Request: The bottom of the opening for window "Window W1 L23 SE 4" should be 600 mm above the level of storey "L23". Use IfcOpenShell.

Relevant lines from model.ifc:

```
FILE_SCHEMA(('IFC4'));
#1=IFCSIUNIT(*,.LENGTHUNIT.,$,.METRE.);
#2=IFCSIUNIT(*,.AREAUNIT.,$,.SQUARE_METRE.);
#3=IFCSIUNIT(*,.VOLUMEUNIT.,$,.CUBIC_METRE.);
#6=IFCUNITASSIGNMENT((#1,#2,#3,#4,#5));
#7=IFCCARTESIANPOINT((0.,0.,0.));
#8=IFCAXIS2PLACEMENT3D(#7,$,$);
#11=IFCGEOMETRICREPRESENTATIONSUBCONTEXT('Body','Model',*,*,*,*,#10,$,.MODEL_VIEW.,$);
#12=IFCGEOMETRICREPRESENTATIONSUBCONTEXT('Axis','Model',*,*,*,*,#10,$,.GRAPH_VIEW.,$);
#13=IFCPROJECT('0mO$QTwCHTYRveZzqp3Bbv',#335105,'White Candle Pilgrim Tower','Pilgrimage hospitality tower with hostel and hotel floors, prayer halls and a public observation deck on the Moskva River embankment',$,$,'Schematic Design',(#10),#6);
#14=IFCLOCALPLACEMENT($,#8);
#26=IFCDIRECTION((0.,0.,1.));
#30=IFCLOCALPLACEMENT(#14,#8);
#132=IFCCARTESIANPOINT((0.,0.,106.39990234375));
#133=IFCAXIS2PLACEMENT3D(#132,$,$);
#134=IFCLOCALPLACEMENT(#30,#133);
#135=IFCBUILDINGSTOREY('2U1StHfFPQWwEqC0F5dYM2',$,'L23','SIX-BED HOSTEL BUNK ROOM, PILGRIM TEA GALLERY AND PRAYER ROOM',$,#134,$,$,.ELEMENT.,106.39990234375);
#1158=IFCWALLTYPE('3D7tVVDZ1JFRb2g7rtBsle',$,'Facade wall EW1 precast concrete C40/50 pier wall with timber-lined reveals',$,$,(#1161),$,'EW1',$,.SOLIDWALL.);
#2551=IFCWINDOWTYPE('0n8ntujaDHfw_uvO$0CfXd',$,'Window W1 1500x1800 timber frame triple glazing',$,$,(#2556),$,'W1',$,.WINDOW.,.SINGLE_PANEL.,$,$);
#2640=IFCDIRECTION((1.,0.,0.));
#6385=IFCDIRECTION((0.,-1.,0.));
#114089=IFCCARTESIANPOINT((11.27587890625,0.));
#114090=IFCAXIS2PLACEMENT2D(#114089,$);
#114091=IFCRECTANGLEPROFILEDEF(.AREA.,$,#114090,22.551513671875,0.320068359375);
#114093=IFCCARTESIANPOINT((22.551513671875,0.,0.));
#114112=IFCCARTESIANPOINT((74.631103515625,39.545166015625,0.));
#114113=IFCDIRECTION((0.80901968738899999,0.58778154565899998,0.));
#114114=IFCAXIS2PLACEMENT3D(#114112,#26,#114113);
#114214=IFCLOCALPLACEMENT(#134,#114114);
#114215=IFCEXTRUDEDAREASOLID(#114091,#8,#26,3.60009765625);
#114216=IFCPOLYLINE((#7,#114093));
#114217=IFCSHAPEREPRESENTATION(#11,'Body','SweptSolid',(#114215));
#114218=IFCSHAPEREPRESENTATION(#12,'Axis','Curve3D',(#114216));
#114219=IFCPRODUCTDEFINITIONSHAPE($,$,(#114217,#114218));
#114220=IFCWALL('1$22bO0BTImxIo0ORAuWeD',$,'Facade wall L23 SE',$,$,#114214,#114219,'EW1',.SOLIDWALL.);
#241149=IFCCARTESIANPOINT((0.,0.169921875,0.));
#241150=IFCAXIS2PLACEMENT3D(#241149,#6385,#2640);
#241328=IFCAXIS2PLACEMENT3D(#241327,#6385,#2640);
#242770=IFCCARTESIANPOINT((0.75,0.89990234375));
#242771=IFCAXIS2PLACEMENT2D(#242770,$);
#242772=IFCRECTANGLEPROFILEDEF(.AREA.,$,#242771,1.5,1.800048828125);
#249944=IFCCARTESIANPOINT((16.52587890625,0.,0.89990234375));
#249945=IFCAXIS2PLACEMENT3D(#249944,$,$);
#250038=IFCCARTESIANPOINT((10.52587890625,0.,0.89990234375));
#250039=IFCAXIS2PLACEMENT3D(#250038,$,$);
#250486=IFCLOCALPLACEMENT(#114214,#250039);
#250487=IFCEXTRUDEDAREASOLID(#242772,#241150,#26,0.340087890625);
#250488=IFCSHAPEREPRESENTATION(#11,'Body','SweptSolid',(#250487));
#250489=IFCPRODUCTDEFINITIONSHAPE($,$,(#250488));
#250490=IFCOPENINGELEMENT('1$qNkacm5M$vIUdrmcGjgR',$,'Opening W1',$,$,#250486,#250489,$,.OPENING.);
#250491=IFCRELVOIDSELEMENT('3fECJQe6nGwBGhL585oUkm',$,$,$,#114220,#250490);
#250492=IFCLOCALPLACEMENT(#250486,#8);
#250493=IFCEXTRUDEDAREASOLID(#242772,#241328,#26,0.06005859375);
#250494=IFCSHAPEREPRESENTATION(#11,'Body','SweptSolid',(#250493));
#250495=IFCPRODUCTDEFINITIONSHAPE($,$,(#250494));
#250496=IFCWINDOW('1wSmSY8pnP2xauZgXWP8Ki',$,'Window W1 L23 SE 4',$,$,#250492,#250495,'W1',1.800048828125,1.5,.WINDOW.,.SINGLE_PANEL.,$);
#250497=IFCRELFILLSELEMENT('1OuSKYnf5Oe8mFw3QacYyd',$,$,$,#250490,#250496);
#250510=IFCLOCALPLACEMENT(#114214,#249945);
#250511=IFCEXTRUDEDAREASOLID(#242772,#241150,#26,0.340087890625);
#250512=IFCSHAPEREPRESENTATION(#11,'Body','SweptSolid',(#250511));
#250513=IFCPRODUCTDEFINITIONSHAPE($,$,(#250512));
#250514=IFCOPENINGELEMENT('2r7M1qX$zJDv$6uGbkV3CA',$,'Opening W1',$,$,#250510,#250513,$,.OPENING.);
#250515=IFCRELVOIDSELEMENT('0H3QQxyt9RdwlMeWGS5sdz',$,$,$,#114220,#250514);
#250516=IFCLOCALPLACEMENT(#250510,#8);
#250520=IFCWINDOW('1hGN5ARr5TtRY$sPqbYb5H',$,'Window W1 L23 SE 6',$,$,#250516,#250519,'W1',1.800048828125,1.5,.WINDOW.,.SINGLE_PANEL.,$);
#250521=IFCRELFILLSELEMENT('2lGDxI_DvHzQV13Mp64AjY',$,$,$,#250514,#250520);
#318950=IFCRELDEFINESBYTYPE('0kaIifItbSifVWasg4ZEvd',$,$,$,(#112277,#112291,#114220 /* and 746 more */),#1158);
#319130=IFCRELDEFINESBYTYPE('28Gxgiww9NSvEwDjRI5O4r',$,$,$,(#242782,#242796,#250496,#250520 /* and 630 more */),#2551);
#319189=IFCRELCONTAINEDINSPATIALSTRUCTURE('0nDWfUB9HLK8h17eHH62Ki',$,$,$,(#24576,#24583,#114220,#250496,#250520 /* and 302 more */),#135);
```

```python
import numpy as np
import ifcopenshell
import ifcopenshell.api.geometry
import ifcopenshell.geom
import ifcopenshell.util.element
import ifcopenshell.util.placement
import ifcopenshell.util.shape
import ifcopenshell.util.unit

model = ifcopenshell.open("model.ifc")
unit_scale = ifcopenshell.util.unit.calculate_unit_scale(model)

window = model.by_id(250496)
opening = window.FillsVoids[0].RelatingOpeningElement
storey = ifcopenshell.util.element.get_container(window, ifc_class="IfcBuildingStorey")
level = ifcopenshell.util.placement.get_local_placement(storey.ObjectPlacement)[2, 3]

# The opening's origin need not be at the sill, so measure its lowest point.
shape = ifcopenshell.geom.create_shape(ifcopenshell.geom.settings(), opening)
bottom = ifcopenshell.util.shape.get_shape_bottom_elevation(shape, shape.geometry) / unit_scale
dz = level + 0.6 / unit_scale - bottom

shift = np.array([0.0, 0.0, dz])
# The window is placed relative to its opening, so it follows when the opening moves.
matrix = ifcopenshell.util.placement.get_local_placement(opening.ObjectPlacement)
matrix[:3, 3] += shift
ifcopenshell.api.geometry.edit_object_placement(
    model, product=opening, matrix=matrix, is_si=False, should_transform_children=True
)

print(f"moved by {dz * unit_scale:+.3f} m")

model.write("model-out.ifc")
```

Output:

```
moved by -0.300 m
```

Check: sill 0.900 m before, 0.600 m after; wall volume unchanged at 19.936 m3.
